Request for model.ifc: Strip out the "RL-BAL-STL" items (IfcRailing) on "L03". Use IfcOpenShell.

First a look at what the model holds.

```python
import ifcopenshell
import ifcopenshell.util.element

model = ifcopenshell.open("model.ifc")
print(model.schema)
storey = next(s for s in model.by_type("IfcBuildingStorey") if s.Name == "L03")
railings = [e for e in ifcopenshell.util.element.get_decomposition(storey) if e.is_a("IfcRailing")]
seen = {}
for e in railings:
    element_type = ifcopenshell.util.element.get_type(e)
    name = element_type.Name if element_type not in (None, e) else None
    seen[name] = seen.get(name, 0) + 1
for name, count in sorted(seen.items(), key=str):
    print(count, "x", name)
```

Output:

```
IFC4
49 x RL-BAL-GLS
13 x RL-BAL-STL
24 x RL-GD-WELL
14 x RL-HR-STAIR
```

```python
import ifcopenshell
import ifcopenshell.api.root
import ifcopenshell.util.element

model = ifcopenshell.open("model.ifc")

storey = next(s for s in model.by_type("IfcBuildingStorey") if s.Name == "L03")
railings = [e for e in ifcopenshell.util.element.get_decomposition(storey) if e.is_a("IfcRailing")]
targets = [e for e in railings if (t := ifcopenshell.util.element.get_type(e)) not in (None, e) and t.Name == "RL-BAL-STL"]

for e in targets:
    ifcopenshell.api.root.remove_product(model, product=e)
print(len(targets), "removed")

model.write("model_rev.ifc")
```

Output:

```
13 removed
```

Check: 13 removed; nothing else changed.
